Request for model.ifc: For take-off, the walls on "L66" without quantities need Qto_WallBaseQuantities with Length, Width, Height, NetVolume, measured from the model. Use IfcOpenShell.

First a look at what the model holds.

```python
import ifcopenshell
import ifcopenshell.util.element
import ifcopenshell.util.unit

model = ifcopenshell.open("model.ifc")
print(model.schema)
for unit_type in ("LENGTHUNIT", "AREAUNIT", "VOLUMEUNIT"):
    print(unit_type, ifcopenshell.util.unit.calculate_unit_scale(model, unit_type))
storey = next(s for s in model.by_type("IfcBuildingStorey") if s.Name == "L66")
walls = [e for e in ifcopenshell.util.element.get_decomposition(storey) if e.is_a("IfcWall")]
for e in sorted(walls, key=lambda e: e.id()):
    print(e.id(), e.is_a(), e.Name, list(ifcopenshell.util.element.get_psets(e, qtos_only=True)), sep=" | ")
```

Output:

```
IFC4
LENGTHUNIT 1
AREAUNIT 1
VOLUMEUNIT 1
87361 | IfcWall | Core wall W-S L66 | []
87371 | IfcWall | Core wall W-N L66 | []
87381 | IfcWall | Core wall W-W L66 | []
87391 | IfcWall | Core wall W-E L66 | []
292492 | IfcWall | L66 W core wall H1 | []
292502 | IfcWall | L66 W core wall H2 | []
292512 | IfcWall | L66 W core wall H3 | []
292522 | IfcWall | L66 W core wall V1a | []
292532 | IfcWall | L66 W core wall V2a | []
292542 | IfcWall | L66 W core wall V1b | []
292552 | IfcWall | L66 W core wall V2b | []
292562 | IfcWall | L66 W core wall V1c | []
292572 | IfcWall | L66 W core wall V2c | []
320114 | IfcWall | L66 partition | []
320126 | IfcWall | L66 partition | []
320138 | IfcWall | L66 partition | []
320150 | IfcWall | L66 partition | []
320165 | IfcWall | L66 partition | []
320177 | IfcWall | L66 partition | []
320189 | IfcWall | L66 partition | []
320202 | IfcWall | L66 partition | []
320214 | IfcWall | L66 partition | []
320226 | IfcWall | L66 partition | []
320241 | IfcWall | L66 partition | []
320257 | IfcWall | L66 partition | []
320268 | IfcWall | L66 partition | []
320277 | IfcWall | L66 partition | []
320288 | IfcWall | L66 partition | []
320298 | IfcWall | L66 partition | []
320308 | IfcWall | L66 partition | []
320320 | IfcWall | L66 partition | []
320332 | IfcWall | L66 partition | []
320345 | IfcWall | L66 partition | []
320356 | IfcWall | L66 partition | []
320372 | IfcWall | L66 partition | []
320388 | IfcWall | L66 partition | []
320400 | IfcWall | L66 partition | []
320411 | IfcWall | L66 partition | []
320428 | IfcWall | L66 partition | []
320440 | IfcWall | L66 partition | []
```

```python
import ifcopenshell
import ifcopenshell.api.pset
import ifcopenshell.geom
import ifcopenshell.util.element
import ifcopenshell.util.shape
import ifcopenshell.util.unit

model = ifcopenshell.open("model.ifc")
unit_scale = ifcopenshell.util.unit.calculate_unit_scale(model)
volume_scale = ifcopenshell.util.unit.calculate_unit_scale(model, "VOLUMEUNIT")
settings = ifcopenshell.geom.settings()

storey = next(s for s in model.by_type("IfcBuildingStorey") if s.Name == "L66")
walls = [e for e in ifcopenshell.util.element.get_decomposition(storey) if e.is_a("IfcWall")]

for e in sorted(walls, key=lambda e: e.id()):
    if ifcopenshell.util.element.get_psets(e, qtos_only=True, should_inherit=False):
        continue
    # Geometry comes back in metres, in the element's own axes.
    shape = ifcopenshell.geom.create_shape(settings, e)
    values = {
        "Length": ifcopenshell.util.shape.get_x(shape.geometry) / unit_scale,
        "Width": ifcopenshell.util.shape.get_y(shape.geometry) / unit_scale,
        "Height": ifcopenshell.util.shape.get_z(shape.geometry) / unit_scale,
        "NetVolume": ifcopenshell.util.shape.get_volume(shape.geometry) / volume_scale,
    }
    qto = ifcopenshell.api.pset.add_qto(model, product=e, name="Qto_WallBaseQuantities")
    ifcopenshell.api.pset.edit_qto(model, qto=qto, properties=values)
    print(e.id(), {k: round(v, 3) for k, v in values.items()})

model.write("model_updated.ifc")
```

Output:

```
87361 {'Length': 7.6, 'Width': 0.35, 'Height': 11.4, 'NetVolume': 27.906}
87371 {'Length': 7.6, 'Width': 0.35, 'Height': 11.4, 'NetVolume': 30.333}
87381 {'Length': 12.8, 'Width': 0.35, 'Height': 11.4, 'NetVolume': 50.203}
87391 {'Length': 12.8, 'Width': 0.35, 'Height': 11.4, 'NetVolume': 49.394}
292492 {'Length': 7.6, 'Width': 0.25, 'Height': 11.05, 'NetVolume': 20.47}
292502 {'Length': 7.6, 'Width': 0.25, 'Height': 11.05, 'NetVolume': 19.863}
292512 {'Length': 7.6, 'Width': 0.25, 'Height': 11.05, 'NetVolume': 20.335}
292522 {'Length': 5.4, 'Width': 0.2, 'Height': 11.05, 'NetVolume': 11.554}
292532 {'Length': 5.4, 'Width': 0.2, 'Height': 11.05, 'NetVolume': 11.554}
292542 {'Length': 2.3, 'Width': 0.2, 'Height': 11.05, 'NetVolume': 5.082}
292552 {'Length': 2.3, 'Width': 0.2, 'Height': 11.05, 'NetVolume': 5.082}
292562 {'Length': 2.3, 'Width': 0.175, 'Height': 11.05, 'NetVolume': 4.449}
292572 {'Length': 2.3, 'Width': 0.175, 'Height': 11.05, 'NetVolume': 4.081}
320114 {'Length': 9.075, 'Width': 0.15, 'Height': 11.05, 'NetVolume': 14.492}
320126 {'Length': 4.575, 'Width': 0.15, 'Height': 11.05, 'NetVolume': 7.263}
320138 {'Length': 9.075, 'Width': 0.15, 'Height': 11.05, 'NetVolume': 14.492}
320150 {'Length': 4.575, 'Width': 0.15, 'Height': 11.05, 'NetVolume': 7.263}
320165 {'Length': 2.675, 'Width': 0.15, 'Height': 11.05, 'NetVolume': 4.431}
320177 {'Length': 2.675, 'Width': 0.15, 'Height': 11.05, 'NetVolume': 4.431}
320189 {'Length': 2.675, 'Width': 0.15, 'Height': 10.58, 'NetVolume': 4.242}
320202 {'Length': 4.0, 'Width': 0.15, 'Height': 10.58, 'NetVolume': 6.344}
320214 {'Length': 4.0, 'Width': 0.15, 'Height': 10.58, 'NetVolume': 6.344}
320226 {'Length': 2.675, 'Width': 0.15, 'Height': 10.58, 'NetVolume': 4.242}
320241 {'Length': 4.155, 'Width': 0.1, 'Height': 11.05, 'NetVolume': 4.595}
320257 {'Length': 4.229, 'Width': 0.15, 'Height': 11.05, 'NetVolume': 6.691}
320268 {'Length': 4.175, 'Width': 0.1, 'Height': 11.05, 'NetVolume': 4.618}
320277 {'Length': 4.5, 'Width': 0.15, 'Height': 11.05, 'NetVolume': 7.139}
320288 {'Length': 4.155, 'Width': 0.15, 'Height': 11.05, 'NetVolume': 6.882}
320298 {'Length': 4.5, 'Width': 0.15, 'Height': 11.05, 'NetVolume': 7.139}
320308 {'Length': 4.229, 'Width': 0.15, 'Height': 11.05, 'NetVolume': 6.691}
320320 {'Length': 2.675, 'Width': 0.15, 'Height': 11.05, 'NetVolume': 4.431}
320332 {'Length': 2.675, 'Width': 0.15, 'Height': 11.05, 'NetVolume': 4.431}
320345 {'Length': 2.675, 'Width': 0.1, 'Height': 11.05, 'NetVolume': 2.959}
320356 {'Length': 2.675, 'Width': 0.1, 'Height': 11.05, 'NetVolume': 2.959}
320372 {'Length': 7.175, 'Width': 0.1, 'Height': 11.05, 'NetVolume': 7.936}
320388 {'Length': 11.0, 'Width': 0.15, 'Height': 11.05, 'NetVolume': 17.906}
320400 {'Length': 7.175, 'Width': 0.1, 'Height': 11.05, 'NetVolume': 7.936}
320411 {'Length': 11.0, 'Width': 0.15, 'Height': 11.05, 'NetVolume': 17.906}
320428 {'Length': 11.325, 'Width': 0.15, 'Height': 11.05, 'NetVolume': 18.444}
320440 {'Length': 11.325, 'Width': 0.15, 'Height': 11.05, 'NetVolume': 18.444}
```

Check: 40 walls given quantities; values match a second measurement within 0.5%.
